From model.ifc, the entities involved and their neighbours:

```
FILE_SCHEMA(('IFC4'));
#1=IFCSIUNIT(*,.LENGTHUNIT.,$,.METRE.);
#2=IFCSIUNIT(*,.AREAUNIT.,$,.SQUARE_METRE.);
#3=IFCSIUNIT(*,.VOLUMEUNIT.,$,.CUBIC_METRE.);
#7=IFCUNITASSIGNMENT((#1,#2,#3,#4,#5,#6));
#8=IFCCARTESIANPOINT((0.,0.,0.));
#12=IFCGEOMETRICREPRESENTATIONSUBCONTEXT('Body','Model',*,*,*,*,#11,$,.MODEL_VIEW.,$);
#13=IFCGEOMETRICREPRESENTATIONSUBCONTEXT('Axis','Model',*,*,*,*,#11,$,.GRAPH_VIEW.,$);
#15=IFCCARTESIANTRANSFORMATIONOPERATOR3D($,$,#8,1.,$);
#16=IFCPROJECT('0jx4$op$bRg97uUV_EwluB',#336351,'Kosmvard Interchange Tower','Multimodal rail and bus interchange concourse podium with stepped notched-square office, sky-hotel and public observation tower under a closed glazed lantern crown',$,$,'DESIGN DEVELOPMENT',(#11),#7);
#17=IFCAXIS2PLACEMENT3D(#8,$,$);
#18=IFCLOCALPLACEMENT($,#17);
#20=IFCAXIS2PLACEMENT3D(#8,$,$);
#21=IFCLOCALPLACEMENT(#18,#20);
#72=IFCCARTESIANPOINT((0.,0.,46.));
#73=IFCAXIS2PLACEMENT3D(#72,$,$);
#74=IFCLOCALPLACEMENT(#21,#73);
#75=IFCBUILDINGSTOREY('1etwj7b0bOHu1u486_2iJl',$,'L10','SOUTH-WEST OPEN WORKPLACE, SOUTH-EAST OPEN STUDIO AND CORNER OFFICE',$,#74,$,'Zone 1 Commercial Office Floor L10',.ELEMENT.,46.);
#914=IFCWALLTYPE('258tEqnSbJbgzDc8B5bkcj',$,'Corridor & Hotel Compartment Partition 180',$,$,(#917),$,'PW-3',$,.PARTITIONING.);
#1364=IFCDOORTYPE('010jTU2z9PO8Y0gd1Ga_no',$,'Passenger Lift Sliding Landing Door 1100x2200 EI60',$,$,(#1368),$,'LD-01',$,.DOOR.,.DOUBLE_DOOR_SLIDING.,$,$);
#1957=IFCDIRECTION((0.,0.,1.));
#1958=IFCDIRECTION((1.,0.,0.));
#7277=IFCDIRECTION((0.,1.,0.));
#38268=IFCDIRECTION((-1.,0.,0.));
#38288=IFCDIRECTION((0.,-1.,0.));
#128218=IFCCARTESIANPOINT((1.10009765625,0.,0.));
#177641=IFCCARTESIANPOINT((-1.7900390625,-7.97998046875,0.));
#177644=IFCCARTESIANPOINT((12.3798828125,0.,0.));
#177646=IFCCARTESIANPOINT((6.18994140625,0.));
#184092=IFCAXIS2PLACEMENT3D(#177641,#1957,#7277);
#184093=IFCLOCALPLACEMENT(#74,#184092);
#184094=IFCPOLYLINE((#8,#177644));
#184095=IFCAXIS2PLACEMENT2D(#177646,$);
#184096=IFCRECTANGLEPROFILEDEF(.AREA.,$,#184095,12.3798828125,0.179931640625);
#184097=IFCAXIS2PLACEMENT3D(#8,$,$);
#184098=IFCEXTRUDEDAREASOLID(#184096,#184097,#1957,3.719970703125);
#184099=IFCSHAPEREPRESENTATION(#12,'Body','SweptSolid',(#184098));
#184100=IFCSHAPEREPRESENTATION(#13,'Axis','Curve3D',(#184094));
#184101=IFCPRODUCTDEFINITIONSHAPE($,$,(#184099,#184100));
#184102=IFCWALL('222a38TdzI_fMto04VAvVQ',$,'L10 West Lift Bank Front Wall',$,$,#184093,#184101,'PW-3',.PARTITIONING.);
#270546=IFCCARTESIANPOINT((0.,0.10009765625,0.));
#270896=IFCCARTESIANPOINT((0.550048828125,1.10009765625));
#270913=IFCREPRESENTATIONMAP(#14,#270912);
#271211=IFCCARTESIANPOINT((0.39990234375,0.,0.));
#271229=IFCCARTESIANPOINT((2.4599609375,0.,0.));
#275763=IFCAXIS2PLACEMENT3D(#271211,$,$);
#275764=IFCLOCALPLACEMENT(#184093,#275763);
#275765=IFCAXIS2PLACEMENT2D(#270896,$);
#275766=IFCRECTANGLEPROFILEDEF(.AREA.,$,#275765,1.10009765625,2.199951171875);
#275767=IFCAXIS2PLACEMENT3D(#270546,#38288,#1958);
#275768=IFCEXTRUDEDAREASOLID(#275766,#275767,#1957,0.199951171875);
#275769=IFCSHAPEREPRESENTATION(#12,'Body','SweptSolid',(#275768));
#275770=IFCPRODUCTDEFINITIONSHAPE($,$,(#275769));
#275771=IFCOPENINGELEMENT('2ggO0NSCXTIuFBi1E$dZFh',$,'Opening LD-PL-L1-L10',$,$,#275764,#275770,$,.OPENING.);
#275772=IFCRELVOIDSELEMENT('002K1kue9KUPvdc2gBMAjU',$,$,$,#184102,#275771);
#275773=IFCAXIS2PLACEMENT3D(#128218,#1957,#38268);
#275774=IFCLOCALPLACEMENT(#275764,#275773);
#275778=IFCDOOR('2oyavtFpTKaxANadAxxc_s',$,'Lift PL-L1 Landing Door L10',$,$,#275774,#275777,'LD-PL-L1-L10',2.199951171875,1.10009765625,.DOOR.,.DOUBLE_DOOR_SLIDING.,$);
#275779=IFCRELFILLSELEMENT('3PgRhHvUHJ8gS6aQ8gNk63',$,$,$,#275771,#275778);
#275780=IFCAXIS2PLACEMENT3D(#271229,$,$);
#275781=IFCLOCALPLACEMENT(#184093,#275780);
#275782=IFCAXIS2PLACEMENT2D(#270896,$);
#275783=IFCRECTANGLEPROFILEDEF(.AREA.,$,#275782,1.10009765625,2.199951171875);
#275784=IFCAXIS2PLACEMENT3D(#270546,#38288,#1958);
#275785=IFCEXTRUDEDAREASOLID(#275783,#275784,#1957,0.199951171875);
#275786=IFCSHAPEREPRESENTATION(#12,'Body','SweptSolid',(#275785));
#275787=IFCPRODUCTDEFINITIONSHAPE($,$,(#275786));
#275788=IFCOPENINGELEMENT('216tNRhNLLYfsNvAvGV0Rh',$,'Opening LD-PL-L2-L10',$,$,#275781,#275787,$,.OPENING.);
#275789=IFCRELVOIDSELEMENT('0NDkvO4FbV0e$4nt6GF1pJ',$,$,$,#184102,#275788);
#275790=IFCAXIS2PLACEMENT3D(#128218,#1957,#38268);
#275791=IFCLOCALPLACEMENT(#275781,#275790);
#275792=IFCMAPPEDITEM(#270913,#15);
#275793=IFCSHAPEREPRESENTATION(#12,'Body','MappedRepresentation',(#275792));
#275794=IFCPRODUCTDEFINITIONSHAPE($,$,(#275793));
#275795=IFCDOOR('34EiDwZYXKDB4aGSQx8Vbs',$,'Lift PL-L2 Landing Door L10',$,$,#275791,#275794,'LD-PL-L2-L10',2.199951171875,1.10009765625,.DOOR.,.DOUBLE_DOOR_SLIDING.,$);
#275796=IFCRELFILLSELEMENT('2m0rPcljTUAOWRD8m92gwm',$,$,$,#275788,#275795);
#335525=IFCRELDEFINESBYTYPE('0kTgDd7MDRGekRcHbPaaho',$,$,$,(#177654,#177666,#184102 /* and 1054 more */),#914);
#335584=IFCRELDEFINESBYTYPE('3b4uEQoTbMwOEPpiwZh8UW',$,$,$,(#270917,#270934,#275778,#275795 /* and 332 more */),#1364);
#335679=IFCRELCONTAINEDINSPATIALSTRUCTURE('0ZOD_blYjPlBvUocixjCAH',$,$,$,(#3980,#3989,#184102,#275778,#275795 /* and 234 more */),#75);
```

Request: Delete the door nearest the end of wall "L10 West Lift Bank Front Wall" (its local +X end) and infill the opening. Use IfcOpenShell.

```python
import ifcopenshell
import ifcopenshell.api.feature
import ifcopenshell.api.root
import ifcopenshell.geom
import ifcopenshell.util.shape

model = ifcopenshell.open("model.ifc")
settings = ifcopenshell.geom.settings()


def volume(element):
    """Net volume in cubic metres, openings subtracted."""
    shape = ifcopenshell.geom.create_shape(settings, element)
    return ifcopenshell.util.shape.get_volume(shape.geometry)


door = model.by_guid("34EiDwZYXKDB4aGSQx8Vbs")
opening = door.FillsVoids[0].RelatingOpeningElement
wall = opening.VoidsElements[0].RelatingBuildingElement
before = volume(wall)

ifcopenshell.api.root.remove_product(model, product=door)
ifcopenshell.api.feature.remove_feature(model, feature=opening)

after = volume(wall)

print(f"wall volume {before:.3f} -> {after:.3f} m3")

model.write("model_v2.ifc")
```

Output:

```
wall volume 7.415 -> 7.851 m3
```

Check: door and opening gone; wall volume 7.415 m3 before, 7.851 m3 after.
